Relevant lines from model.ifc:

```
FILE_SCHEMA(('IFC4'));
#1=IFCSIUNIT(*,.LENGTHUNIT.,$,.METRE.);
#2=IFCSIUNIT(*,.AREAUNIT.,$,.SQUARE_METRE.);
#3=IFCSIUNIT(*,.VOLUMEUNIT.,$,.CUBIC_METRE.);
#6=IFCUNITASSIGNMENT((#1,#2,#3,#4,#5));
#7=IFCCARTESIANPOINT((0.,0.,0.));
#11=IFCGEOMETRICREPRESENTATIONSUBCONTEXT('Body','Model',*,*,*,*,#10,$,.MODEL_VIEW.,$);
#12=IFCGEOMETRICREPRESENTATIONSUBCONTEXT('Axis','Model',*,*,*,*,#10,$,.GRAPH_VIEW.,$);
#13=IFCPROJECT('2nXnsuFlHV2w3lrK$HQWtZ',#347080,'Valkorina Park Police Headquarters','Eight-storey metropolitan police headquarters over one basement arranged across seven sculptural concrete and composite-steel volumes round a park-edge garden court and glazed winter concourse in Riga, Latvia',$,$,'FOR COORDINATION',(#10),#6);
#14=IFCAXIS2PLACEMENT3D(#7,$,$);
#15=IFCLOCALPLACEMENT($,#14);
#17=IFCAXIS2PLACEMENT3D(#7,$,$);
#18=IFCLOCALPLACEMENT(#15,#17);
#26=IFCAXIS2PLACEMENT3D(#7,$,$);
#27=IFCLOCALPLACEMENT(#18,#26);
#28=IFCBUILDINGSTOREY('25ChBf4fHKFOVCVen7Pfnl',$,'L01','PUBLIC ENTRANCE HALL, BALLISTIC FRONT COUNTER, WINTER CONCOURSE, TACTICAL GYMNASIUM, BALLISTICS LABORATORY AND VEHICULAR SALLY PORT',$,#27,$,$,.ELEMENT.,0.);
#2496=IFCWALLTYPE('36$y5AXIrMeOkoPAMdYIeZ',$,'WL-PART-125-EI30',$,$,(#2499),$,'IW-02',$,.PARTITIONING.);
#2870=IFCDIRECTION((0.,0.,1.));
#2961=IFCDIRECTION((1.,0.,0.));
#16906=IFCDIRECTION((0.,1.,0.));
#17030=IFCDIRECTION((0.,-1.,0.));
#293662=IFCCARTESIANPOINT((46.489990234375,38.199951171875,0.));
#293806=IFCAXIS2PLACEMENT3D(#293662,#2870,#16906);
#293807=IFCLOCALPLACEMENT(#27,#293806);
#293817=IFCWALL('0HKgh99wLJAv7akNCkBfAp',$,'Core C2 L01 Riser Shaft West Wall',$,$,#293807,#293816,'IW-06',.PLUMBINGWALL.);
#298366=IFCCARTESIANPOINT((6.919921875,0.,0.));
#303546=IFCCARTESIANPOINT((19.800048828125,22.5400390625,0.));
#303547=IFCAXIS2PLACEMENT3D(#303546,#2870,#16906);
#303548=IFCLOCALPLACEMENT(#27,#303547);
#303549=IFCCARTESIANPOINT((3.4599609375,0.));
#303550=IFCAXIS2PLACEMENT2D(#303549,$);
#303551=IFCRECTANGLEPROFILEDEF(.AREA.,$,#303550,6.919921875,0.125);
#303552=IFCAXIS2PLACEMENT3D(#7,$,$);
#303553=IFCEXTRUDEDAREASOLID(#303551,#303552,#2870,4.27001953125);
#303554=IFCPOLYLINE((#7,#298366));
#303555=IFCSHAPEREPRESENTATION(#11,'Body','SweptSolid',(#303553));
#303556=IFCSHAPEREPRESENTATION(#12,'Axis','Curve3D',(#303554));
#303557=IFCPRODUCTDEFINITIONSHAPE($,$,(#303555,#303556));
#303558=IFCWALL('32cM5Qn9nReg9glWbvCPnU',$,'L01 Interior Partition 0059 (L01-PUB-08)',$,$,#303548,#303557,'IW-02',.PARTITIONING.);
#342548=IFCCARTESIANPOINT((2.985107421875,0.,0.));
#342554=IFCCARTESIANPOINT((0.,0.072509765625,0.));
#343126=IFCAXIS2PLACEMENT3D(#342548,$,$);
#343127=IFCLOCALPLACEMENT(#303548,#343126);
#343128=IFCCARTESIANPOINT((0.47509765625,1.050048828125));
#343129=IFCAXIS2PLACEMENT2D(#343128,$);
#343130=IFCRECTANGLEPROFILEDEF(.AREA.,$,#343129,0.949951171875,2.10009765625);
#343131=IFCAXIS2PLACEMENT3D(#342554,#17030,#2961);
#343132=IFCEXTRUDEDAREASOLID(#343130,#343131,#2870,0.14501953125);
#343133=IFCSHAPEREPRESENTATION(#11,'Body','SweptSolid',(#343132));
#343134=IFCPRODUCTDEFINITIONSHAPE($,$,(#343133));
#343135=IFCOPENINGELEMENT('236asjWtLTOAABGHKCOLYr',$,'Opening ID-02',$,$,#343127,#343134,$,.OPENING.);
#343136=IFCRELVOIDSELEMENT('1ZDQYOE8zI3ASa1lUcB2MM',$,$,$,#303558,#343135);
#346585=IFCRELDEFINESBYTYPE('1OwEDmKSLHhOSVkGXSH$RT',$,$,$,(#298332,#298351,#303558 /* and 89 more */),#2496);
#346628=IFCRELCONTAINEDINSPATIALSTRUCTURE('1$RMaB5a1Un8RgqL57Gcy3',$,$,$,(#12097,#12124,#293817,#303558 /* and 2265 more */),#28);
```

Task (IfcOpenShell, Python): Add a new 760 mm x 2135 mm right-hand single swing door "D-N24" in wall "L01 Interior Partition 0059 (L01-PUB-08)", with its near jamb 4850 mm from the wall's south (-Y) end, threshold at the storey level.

```python
import numpy as np
import ifcopenshell
import ifcopenshell.api.feature
import ifcopenshell.api.geometry
import ifcopenshell.api.root
import ifcopenshell.api.spatial
import ifcopenshell.geom
import ifcopenshell.util.element
import ifcopenshell.util.placement
import ifcopenshell.util.representation
import ifcopenshell.util.shape
import ifcopenshell.util.unit

model = ifcopenshell.open("model.ifc")
unit_scale = ifcopenshell.util.unit.calculate_unit_scale(model)
settings = ifcopenshell.geom.settings()


def volume(element):
    """Net volume in cubic metres, openings subtracted."""
    shape = ifcopenshell.geom.create_shape(settings, element)
    return ifcopenshell.util.shape.get_volume(shape.geometry)


wall = model.by_guid("32cM5Qn9nReg9glWbvCPnU")
storey = ifcopenshell.util.element.get_container(wall, ifc_class="IfcBuildingStorey")
context = ifcopenshell.util.representation.get_context(model, "Model", "Body", "MODEL_VIEW")
before = volume(wall)

width, height, from_end, sill = 0.76, 2.135, 4.85, 0.0  # metres

# The wall runs along its own X axis, and the end named is its -X end.
wall_shape = ifcopenshell.geom.create_shape(settings, wall)
x, y, z = ifcopenshell.util.shape.get_vertices(wall_shape.geometry).T
start = x.min() + from_end
face, thickness = float(y.min()), float(y.max() - y.min())
wall_matrix = ifcopenshell.util.placement.get_local_placement(wall.ObjectPlacement)
level = ifcopenshell.util.placement.get_local_placement(storey.ObjectPlacement)[2, 3]


def in_wall(x, y):
    """Placement at x, y metres in the wall's axes, at sill height."""
    matrix = wall_matrix.copy()
    matrix[:, 3] = wall_matrix @ np.array([x / unit_scale, y / unit_scale, 0.0, 1.0])
    matrix[2, 3] = level + sill / unit_scale
    return matrix


# Opening: a box that overshoots both wall faces by 50 mm.
opening = ifcopenshell.api.root.create_entity(model, ifc_class="IfcOpeningElement", predefined_type="OPENING")
box = ifcopenshell.api.geometry.add_wall_representation(
    model, context=context, length=width, height=height, thickness=thickness + 0.1
)
ifcopenshell.api.geometry.assign_representation(model, product=opening, representation=box)
ifcopenshell.api.geometry.edit_object_placement(model, product=opening, matrix=in_wall(start, face - 0.05), is_si=False)
ifcopenshell.api.feature.add_feature(model, feature=opening, element=wall)

door = ifcopenshell.api.root.create_entity(model, ifc_class="IfcDoor", name="D-N24", predefined_type="DOOR")
door.OverallWidth, door.OverallHeight = width / unit_scale, height / unit_scale
door.OperationType = "SINGLE_SWING_RIGHT"
body = ifcopenshell.api.geometry.add_door_representation(
    model,
    context=context,
    overall_width=door.OverallWidth,
    overall_height=door.OverallHeight,
    operation_type="SINGLE_SWING_RIGHT",
    lining_properties={"LiningDepth": thickness / unit_scale, "ThresholdDepth": thickness / unit_scale},
)
ifcopenshell.api.geometry.assign_representation(model, product=door, representation=body)
ifcopenshell.api.spatial.assign_container(model, products=[door], relating_structure=storey)
ifcopenshell.api.feature.add_filling(model, opening=opening, element=door)

# The lining spans the wall, so the door starts at the wall face.
ifcopenshell.api.geometry.edit_object_placement(model, product=door, matrix=in_wall(start, face), is_si=False)

after = volume(wall)

print(f"wall volume {before:.3f} -> {after:.3f} m3")

model.write("model_updated.ifc")
```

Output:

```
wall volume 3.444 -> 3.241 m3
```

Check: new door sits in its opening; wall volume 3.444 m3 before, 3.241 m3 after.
